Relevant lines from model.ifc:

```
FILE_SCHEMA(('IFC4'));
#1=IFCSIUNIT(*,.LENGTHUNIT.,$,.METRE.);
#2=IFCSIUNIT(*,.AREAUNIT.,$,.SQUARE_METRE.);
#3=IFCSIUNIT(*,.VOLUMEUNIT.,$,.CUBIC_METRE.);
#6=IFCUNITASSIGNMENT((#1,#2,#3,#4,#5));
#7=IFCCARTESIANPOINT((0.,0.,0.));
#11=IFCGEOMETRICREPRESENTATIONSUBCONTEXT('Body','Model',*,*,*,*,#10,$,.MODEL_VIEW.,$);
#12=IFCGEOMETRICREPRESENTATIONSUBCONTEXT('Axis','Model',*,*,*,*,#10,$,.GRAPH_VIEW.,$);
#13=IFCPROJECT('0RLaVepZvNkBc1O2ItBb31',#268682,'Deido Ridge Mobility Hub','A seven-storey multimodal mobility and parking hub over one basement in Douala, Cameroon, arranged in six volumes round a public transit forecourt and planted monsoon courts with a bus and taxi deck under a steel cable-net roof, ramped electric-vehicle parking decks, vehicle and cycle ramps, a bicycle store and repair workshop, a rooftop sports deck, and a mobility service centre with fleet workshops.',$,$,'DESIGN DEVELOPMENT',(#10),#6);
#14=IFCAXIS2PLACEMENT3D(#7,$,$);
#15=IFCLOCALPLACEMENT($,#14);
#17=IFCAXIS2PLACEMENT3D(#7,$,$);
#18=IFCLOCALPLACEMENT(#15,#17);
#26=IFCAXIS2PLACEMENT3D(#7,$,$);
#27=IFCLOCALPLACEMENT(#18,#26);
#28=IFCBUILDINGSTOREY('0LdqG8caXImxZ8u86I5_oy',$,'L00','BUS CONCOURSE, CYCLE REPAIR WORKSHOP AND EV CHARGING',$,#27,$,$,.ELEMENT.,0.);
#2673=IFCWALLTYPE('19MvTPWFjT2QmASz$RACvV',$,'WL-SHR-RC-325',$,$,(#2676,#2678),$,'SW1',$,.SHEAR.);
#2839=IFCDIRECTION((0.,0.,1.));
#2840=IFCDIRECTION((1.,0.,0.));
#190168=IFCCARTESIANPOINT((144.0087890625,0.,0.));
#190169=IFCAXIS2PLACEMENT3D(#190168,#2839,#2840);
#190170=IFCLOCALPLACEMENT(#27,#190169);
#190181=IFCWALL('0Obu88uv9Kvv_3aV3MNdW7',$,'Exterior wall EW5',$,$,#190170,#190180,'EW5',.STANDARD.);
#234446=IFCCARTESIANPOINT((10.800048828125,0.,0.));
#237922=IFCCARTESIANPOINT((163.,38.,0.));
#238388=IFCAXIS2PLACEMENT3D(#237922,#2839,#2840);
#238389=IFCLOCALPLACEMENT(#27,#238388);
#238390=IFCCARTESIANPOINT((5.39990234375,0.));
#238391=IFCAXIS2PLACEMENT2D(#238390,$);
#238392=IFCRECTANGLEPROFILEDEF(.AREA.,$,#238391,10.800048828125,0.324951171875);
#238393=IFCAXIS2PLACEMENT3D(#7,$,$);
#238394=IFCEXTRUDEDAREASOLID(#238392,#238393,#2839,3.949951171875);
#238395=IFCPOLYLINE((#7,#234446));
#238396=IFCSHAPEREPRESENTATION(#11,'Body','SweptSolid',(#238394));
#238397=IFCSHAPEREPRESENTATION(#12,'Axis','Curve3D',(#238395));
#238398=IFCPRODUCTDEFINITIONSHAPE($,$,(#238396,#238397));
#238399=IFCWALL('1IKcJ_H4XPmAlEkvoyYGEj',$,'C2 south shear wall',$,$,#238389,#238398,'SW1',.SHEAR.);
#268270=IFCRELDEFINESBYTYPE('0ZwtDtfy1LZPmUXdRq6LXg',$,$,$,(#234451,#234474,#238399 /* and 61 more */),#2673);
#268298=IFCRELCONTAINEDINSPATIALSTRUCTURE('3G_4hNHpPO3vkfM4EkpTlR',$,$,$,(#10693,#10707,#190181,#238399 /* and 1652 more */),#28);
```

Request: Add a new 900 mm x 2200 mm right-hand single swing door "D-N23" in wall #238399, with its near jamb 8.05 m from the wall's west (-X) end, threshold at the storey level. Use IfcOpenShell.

```python
import numpy as np
import ifcopenshell
import ifcopenshell.api.feature
import ifcopenshell.api.geometry
import ifcopenshell.api.root
import ifcopenshell.api.spatial
import ifcopenshell.geom
import ifcopenshell.util.element
import ifcopenshell.util.placement
import ifcopenshell.util.representation
import ifcopenshell.util.shape
import ifcopenshell.util.unit

model = ifcopenshell.open("model.ifc")
unit_scale = ifcopenshell.util.unit.calculate_unit_scale(model)
settings = ifcopenshell.geom.settings()


def volume(element):
    """Net volume in cubic metres, openings subtracted."""
    shape = ifcopenshell.geom.create_shape(settings, element)
    return ifcopenshell.util.shape.get_volume(shape.geometry)


wall = model.by_guid("1IKcJ_H4XPmAlEkvoyYGEj")
storey = ifcopenshell.util.element.get_container(wall, ifc_class="IfcBuildingStorey")
context = ifcopenshell.util.representation.get_context(model, "Model", "Body", "MODEL_VIEW")
before = volume(wall)

width, height, from_end, sill = 0.9, 2.2, 8.05, 0.0  # metres

# The wall runs along its own X axis, and the end named is its -X end.
wall_shape = ifcopenshell.geom.create_shape(settings, wall)
x, y, z = ifcopenshell.util.shape.get_vertices(wall_shape.geometry).T
start = x.min() + from_end
face, thickness = float(y.min()), float(y.max() - y.min())
wall_matrix = ifcopenshell.util.placement.get_local_placement(wall.ObjectPlacement)
level = ifcopenshell.util.placement.get_local_placement(storey.ObjectPlacement)[2, 3]


def in_wall(x, y):
    """Placement at x, y metres in the wall's axes, at sill height."""
    matrix = wall_matrix.copy()
    matrix[:, 3] = wall_matrix @ np.array([x / unit_scale, y / unit_scale, 0.0, 1.0])
    matrix[2, 3] = level + sill / unit_scale
    return matrix


# Opening: a box that overshoots both wall faces by 50 mm.
opening = ifcopenshell.api.root.create_entity(model, ifc_class="IfcOpeningElement", predefined_type="OPENING")
box = ifcopenshell.api.geometry.add_wall_representation(
    model, context=context, length=width, height=height, thickness=thickness + 0.1
)
ifcopenshell.api.geometry.assign_representation(model, product=opening, representation=box)
ifcopenshell.api.geometry.edit_object_placement(model, product=opening, matrix=in_wall(start, face - 0.05), is_si=False)
ifcopenshell.api.feature.add_feature(model, feature=opening, element=wall)

door = ifcopenshell.api.root.create_entity(model, ifc_class="IfcDoor", name="D-N23", predefined_type="DOOR")
door.OverallWidth, door.OverallHeight = width / unit_scale, height / unit_scale
door.OperationType = "SINGLE_SWING_RIGHT"
body = ifcopenshell.api.geometry.add_door_representation(
    model,
    context=context,
    overall_width=door.OverallWidth,
    overall_height=door.OverallHeight,
    operation_type="SINGLE_SWING_RIGHT",
    lining_properties={"LiningDepth": thickness / unit_scale, "ThresholdDepth": thickness / unit_scale},
)
ifcopenshell.api.geometry.assign_representation(model, product=door, representation=body)
ifcopenshell.api.spatial.assign_container(model, products=[door], relating_structure=storey)
ifcopenshell.api.feature.add_filling(model, opening=opening, element=door)

# The lining spans the wall, so the door starts at the wall face.
ifcopenshell.api.geometry.edit_object_placement(model, product=door, matrix=in_wall(start, face), is_si=False)

after = volume(wall)

print(f"wall volume {before:.3f} -> {after:.3f} m3")

model.write("model_v2.ifc")
```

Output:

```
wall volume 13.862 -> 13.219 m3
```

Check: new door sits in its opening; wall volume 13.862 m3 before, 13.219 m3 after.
